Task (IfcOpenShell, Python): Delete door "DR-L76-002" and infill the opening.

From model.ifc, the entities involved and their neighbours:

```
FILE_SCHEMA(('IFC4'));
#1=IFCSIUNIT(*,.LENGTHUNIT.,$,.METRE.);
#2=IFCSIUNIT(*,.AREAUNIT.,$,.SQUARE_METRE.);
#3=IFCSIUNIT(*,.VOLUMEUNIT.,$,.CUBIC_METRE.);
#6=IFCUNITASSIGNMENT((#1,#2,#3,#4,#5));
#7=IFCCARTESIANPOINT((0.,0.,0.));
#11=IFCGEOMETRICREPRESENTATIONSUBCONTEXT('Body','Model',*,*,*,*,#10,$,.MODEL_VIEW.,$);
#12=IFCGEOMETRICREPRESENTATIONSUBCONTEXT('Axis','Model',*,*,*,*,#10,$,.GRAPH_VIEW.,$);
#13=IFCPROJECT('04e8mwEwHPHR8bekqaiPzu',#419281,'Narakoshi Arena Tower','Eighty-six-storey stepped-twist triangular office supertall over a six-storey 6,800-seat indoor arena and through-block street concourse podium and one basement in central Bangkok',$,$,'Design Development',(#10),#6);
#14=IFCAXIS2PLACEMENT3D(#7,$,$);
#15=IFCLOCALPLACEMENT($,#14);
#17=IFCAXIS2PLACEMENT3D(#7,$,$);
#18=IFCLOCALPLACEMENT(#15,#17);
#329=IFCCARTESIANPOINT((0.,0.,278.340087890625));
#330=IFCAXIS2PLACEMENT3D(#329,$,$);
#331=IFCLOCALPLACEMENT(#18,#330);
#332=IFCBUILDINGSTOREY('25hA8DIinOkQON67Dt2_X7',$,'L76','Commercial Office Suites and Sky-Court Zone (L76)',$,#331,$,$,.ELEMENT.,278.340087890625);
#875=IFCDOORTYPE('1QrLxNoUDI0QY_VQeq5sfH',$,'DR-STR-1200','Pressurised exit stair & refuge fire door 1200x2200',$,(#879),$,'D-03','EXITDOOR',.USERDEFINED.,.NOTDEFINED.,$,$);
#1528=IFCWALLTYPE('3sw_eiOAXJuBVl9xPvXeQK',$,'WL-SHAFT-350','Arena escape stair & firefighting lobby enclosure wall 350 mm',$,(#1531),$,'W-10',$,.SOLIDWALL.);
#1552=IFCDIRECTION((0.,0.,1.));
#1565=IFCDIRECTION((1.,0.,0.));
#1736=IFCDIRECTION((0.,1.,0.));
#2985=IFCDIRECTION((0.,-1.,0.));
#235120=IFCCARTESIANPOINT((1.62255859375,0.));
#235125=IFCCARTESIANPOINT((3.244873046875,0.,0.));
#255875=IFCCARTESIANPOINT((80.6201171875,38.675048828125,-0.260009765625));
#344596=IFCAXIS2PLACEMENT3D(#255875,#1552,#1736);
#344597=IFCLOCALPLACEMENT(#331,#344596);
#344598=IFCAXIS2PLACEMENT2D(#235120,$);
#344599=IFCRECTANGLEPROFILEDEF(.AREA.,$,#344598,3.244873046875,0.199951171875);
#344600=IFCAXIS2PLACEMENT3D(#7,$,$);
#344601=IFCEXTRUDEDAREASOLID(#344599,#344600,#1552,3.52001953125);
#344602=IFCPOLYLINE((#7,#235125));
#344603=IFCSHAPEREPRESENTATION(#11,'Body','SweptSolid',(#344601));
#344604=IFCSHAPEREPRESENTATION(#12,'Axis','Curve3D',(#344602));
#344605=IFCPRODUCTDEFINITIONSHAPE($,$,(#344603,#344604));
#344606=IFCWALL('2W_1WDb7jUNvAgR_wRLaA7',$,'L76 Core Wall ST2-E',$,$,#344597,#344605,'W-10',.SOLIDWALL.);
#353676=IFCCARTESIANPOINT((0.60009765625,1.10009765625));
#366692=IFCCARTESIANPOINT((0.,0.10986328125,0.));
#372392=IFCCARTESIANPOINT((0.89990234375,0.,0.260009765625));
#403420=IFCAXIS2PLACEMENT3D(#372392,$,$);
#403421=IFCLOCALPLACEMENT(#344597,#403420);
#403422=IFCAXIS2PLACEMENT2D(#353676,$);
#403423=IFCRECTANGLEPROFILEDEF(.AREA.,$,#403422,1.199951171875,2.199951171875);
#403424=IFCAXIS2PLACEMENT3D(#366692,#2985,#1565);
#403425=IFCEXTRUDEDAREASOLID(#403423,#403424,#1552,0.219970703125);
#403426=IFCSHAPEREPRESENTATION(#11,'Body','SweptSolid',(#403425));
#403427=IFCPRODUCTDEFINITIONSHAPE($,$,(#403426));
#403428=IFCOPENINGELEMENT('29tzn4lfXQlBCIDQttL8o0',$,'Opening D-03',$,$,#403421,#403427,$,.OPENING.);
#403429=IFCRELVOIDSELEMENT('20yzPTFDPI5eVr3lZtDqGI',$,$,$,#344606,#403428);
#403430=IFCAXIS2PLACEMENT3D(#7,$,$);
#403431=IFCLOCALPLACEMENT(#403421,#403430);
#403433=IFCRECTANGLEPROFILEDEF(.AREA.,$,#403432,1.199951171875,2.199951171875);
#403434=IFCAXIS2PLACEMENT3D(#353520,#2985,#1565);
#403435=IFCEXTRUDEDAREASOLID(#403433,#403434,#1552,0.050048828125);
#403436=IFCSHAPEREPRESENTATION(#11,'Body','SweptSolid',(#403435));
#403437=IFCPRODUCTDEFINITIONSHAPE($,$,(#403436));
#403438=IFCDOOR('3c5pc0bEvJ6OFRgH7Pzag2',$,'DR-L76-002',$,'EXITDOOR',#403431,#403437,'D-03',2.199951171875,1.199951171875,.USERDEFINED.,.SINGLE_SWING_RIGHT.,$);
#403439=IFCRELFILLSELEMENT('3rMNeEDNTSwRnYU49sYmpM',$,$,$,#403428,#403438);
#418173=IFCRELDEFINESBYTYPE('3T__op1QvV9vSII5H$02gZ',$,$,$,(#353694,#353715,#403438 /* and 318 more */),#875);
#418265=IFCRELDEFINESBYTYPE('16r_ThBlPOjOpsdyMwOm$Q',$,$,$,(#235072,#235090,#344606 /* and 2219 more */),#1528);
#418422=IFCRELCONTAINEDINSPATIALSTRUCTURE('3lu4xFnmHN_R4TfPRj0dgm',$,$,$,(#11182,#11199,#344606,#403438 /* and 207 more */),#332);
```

```python
import ifcopenshell
import ifcopenshell.api.feature
import ifcopenshell.api.root
import ifcopenshell.geom
import ifcopenshell.util.shape

model = ifcopenshell.open("model.ifc")
settings = ifcopenshell.geom.settings()


def volume(element):
    """Net volume in cubic metres, openings subtracted."""
    shape = ifcopenshell.geom.create_shape(settings, element)
    return ifcopenshell.util.shape.get_volume(shape.geometry)


door = model.by_id(403438)
opening = door.FillsVoids[0].RelatingOpeningElement
wall = opening.VoidsElements[0].RelatingBuildingElement
before = volume(wall)

ifcopenshell.api.root.remove_product(model, product=door)
ifcopenshell.api.feature.remove_feature(model, feature=opening)

after = volume(wall)

print(f"wall volume {before:.3f} -> {after:.3f} m3")

model.write("model_rev.ifc")
```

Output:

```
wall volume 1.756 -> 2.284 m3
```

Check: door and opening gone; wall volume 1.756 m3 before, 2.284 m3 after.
